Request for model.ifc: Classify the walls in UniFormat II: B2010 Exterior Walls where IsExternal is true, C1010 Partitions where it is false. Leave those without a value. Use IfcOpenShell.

First a look at what the model holds.

```python
import ifcopenshell
import ifcopenshell.util.element

model = ifcopenshell.open("model.ifc")
print(model.schema)
print("classifications:", [c.Name for c in model.by_type("IfcClassification")])
values = [ifcopenshell.util.element.get_pset(e, "Pset_WallCommon", "IsExternal") for e in model.by_type("IfcWall")]
for value in (True, False, None):
    print("IsExternal", value, values.count(value))
```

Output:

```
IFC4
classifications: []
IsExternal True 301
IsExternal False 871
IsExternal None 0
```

```python
import ifcopenshell
import ifcopenshell.api.classification
import ifcopenshell.util.element

model = ifcopenshell.open("model.ifc")

system = ifcopenshell.api.classification.add_classification(model, classification="UniFormat II")

walls = model.by_type("IfcWall")
external = {e: ifcopenshell.util.element.get_pset(e, "Pset_WallCommon", "IsExternal") for e in walls}
for flag, code, name in ((True, "B2010", "Exterior Walls"), (False, "C1010", "Partitions")):
    products = [e for e in walls if external[e] is flag]
    ifcopenshell.api.classification.add_reference(
        model, products=products, classification=system, identification=code, name=name
    )
    print(code, len(products))

model.write("model-out.ifc")
```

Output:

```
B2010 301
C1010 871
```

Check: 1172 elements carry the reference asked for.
